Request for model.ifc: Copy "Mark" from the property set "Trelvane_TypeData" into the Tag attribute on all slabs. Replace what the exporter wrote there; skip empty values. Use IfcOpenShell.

First a look at what the model holds.

```python
import ifcopenshell
import ifcopenshell.util.element

model = ifcopenshell.open("model.ifc")
print(model.schema)
slabs = model.by_type("IfcSlab")
print(len(slabs), "slabs")
for e in slabs[:8]:
    source = ifcopenshell.util.element.get_pset(e, "Trelvane_TypeData", "Mark")
    target = e.Tag
    print(e.id(), repr(source), repr(target), sep=" | ")
```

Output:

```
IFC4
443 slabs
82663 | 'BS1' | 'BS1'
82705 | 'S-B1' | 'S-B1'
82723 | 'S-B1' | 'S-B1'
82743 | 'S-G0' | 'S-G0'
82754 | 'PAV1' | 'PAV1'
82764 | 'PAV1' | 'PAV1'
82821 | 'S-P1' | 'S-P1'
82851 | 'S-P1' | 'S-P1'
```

```python
import ifcopenshell
import ifcopenshell.util.element

model = ifcopenshell.open("model.ifc")

count = 0
for e in model.by_type("IfcSlab"):
    value = ifcopenshell.util.element.get_pset(e, "Trelvane_TypeData", "Mark")
    current = e.Tag
    if not value or not value.strip() or current == value:
        continue
    e.Tag = value
    count += 1

print(count, "slabs updated")

model.write("model_updated.ifc")
```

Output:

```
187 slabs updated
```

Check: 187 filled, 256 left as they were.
